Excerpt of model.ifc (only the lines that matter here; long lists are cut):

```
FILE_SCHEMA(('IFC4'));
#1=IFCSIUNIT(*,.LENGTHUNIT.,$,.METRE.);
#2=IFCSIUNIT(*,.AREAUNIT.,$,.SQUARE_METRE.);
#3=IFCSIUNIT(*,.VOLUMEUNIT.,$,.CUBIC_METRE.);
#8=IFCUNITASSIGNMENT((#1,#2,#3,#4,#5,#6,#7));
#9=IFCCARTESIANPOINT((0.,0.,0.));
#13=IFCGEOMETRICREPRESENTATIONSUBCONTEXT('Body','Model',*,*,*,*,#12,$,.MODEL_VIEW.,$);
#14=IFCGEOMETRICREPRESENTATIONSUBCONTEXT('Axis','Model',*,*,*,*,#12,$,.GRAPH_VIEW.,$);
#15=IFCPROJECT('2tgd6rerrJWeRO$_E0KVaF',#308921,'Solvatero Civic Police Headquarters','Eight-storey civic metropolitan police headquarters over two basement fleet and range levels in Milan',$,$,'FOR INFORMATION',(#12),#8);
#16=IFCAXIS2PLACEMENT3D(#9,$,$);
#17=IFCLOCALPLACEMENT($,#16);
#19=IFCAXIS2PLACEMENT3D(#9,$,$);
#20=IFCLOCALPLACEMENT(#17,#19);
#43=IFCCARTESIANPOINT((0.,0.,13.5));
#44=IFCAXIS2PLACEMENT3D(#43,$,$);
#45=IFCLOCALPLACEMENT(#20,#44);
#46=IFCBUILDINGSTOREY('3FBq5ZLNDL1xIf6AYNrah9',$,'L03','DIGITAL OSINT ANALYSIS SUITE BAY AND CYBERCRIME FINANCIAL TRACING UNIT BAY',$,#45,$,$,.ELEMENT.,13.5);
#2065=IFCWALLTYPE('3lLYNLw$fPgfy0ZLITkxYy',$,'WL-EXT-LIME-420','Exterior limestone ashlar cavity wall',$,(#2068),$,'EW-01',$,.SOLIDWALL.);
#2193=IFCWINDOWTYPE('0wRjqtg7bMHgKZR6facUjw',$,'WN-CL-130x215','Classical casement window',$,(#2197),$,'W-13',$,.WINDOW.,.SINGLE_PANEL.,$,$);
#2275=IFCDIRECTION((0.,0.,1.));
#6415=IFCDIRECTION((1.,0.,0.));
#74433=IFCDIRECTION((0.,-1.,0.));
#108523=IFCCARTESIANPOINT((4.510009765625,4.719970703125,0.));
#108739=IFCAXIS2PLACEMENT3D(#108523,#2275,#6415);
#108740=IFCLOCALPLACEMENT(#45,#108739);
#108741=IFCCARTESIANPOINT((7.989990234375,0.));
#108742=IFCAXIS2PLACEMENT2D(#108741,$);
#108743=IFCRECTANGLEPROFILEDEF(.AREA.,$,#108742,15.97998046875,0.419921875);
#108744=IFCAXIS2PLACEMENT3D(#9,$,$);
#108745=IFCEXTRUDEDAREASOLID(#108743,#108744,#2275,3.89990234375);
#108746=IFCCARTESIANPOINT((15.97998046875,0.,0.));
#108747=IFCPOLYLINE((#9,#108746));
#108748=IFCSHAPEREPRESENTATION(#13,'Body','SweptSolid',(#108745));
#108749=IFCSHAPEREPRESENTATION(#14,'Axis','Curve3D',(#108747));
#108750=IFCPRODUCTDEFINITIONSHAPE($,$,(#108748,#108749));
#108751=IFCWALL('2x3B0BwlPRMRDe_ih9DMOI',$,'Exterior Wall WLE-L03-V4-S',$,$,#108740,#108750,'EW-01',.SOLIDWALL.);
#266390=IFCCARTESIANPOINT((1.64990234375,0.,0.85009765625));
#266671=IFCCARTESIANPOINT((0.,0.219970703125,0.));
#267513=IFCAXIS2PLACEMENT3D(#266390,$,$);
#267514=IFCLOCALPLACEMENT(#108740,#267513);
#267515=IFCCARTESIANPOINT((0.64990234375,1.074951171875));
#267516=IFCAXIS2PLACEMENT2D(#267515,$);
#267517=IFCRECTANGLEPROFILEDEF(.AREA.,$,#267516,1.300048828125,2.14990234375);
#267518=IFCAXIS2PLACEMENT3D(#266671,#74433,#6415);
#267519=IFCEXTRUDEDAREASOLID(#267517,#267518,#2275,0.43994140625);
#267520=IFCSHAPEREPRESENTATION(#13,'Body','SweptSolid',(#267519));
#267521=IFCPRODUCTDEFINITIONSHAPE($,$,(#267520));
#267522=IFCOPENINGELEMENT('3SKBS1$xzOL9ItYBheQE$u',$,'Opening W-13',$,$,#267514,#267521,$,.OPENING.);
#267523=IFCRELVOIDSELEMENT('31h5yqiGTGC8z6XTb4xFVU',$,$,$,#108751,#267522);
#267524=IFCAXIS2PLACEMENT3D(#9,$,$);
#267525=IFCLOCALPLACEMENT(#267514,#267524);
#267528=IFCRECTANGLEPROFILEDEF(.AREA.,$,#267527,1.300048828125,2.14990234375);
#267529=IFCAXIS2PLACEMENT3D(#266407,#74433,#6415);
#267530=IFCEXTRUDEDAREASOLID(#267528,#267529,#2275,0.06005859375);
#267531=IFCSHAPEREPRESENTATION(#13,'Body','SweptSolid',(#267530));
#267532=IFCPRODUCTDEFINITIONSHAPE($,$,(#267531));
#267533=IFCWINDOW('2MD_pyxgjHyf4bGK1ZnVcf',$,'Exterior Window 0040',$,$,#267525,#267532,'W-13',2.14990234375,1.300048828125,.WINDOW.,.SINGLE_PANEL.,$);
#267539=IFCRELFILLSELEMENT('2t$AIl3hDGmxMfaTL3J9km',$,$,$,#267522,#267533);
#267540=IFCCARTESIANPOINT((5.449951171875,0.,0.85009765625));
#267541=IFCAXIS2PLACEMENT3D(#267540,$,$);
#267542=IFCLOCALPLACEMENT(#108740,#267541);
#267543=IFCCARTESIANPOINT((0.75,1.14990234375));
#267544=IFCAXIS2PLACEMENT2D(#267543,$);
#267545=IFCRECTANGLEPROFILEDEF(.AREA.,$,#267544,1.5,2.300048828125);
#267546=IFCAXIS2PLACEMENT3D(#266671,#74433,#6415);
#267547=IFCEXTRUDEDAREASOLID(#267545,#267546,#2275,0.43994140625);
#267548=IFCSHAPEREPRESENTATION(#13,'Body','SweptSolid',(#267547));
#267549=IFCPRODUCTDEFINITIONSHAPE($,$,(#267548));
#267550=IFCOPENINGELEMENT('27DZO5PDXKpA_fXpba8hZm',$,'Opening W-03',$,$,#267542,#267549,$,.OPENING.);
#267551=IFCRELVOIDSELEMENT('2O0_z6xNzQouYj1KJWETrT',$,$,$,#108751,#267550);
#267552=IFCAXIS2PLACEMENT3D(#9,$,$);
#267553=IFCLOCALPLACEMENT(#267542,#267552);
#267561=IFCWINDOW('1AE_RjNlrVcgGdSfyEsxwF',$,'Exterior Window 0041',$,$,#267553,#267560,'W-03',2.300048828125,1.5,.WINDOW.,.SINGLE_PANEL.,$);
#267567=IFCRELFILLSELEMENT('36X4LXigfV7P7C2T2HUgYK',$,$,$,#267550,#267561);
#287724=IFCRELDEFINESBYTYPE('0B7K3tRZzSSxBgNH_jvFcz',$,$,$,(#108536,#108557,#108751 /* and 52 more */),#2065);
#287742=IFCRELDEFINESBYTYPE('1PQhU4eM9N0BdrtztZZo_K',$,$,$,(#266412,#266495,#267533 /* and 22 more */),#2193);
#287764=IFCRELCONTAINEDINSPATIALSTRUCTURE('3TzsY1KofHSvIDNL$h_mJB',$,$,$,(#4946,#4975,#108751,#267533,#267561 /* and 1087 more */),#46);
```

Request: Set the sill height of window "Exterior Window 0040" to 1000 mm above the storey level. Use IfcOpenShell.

```python
import numpy as np
import ifcopenshell
import ifcopenshell.api.geometry
import ifcopenshell.geom
import ifcopenshell.util.element
import ifcopenshell.util.placement
import ifcopenshell.util.shape
import ifcopenshell.util.unit

model = ifcopenshell.open("model.ifc")
unit_scale = ifcopenshell.util.unit.calculate_unit_scale(model)

window = model.by_id(267533)
opening = window.FillsVoids[0].RelatingOpeningElement
storey = ifcopenshell.util.element.get_container(window, ifc_class="IfcBuildingStorey")
level = ifcopenshell.util.placement.get_local_placement(storey.ObjectPlacement)[2, 3]

# The opening's origin need not be at the sill, so measure its lowest point.
shape = ifcopenshell.geom.create_shape(ifcopenshell.geom.settings(), opening)
bottom = ifcopenshell.util.shape.get_shape_bottom_elevation(shape, shape.geometry) / unit_scale
dz = level + 1 / unit_scale - bottom

shift = np.array([0.0, 0.0, dz])
# The window is placed relative to its opening, so it follows when the opening moves.
matrix = ifcopenshell.util.placement.get_local_placement(opening.ObjectPlacement)
matrix[:3, 3] += shift
ifcopenshell.api.geometry.edit_object_placement(
    model, product=opening, matrix=matrix, is_si=False, should_transform_children=True
)

print(f"moved by {dz * unit_scale:+.3f} m")

model.write("model_rev.ifc")
```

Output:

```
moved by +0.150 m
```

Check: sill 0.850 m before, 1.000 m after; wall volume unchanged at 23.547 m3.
